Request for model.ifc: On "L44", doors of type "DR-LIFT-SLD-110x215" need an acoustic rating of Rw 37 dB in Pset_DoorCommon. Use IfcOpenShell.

First a look at what the model holds.

```python
import ifcopenshell
import ifcopenshell.util.element

model = ifcopenshell.open("model.ifc")
print(model.schema)
storey = next(s for s in model.by_type("IfcBuildingStorey") if s.Name == "L44")
doors = [e for e in ifcopenshell.util.element.get_decomposition(storey) if e.is_a("IfcDoor")]
seen = {}
for e in doors:
    element_type = ifcopenshell.util.element.get_type(e)
    key = (element_type.Name if element_type != e and element_type else None, ifcopenshell.util.element.get_pset(e, "Pset_DoorCommon", "AcousticRating"))
    seen[key] = seen.get(key, 0) + 1
for (name, value), count in sorted(seen.items(), key=str):
    print(count, "x", name, "|", value)
```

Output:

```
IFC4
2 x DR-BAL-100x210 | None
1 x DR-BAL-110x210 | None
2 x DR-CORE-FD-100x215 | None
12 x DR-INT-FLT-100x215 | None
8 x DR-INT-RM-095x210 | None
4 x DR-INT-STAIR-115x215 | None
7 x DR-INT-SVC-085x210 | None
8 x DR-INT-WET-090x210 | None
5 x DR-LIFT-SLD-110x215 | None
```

```python
import ifcopenshell
import ifcopenshell.api.pset
import ifcopenshell.util.element

model = ifcopenshell.open("model.ifc")

storey = next(s for s in model.by_type("IfcBuildingStorey") if s.Name == "L44")
doors = [e for e in ifcopenshell.util.element.get_decomposition(storey) if e.is_a("IfcDoor")]

count = 0
for e in doors:
    element_type = ifcopenshell.util.element.get_type(e)
    if element_type in (None, e) or element_type.Name != "DR-LIFT-SLD-110x215":
        continue
    # add_pset returns the element's existing set when there is one.
    pset = ifcopenshell.api.pset.add_pset(model, product=e, name="Pset_DoorCommon")
    ifcopenshell.api.pset.edit_pset(model, pset=pset, properties={"AcousticRating": "Rw 37 dB"})
    count += 1

print(count, "doors updated")

model.write("model_updated.ifc")
```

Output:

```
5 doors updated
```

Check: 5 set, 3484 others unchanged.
